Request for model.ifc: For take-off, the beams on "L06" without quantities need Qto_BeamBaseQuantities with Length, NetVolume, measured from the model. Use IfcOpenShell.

First a look at what the model holds.

```python
import ifcopenshell
import ifcopenshell.util.element
import ifcopenshell.util.unit

model = ifcopenshell.open("model.ifc")
print(model.schema)
for unit_type in ("LENGTHUNIT", "AREAUNIT", "VOLUMEUNIT"):
    print(unit_type, ifcopenshell.util.unit.calculate_unit_scale(model, unit_type))
storey = next(s for s in model.by_type("IfcBuildingStorey") if s.Name == "L06")
beams = [e for e in ifcopenshell.util.element.get_decomposition(storey) if e.is_a("IfcBeam")]
for e in sorted(beams, key=lambda e: e.id()):
    print(e.id(), e.is_a(), e.Name, list(ifcopenshell.util.element.get_psets(e, qtos_only=True)), sep=" | ")
```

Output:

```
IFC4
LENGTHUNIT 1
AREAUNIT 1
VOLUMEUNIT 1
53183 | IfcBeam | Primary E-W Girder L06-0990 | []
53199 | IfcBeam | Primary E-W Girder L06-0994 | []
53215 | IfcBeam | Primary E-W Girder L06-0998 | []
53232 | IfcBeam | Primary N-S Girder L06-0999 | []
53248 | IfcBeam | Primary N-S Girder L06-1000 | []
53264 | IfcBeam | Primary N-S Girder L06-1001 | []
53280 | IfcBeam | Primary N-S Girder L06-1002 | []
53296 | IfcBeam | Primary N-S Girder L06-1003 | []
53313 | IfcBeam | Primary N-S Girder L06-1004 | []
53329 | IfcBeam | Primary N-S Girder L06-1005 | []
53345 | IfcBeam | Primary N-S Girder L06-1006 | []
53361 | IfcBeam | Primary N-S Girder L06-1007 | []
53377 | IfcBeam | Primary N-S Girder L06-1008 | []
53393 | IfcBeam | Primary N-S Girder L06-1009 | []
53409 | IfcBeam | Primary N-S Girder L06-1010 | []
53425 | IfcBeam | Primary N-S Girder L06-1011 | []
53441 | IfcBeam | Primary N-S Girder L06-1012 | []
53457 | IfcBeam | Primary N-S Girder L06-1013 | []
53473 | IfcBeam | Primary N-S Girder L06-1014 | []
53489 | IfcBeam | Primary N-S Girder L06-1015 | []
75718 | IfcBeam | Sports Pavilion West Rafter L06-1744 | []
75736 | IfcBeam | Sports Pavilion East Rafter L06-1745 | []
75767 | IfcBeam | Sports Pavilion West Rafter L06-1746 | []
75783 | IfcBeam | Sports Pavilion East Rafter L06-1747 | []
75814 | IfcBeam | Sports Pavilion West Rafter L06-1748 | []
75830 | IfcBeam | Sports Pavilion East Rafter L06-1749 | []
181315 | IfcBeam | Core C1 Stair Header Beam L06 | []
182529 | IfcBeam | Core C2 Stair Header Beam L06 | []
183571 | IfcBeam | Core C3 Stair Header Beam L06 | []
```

```python
import ifcopenshell
import ifcopenshell.api.pset
import ifcopenshell.geom
import ifcopenshell.util.element
import ifcopenshell.util.shape
import ifcopenshell.util.unit

model = ifcopenshell.open("model.ifc")
unit_scale = ifcopenshell.util.unit.calculate_unit_scale(model)
volume_scale = ifcopenshell.util.unit.calculate_unit_scale(model, "VOLUMEUNIT")
settings = ifcopenshell.geom.settings()

storey = next(s for s in model.by_type("IfcBuildingStorey") if s.Name == "L06")
beams = [e for e in ifcopenshell.util.element.get_decomposition(storey) if e.is_a("IfcBeam")]

for e in sorted(beams, key=lambda e: e.id()):
    if ifcopenshell.util.element.get_psets(e, qtos_only=True, should_inherit=False):
        continue
    # Geometry comes back in metres, in the element's own axes.
    shape = ifcopenshell.geom.create_shape(settings, e)
    values = {
        "Length": ifcopenshell.util.shape.get_max_xyz(shape.geometry) / unit_scale,
        "NetVolume": ifcopenshell.util.shape.get_volume(shape.geometry) / volume_scale,
    }
    qto = ifcopenshell.api.pset.add_qto(model, product=e, name="Qto_BeamBaseQuantities")
    ifcopenshell.api.pset.edit_qto(model, qto=qto, properties=values)
    print(e.id(), {k: round(v, 3) for k, v in values.items()})

model.write("model_rev.ifc")
```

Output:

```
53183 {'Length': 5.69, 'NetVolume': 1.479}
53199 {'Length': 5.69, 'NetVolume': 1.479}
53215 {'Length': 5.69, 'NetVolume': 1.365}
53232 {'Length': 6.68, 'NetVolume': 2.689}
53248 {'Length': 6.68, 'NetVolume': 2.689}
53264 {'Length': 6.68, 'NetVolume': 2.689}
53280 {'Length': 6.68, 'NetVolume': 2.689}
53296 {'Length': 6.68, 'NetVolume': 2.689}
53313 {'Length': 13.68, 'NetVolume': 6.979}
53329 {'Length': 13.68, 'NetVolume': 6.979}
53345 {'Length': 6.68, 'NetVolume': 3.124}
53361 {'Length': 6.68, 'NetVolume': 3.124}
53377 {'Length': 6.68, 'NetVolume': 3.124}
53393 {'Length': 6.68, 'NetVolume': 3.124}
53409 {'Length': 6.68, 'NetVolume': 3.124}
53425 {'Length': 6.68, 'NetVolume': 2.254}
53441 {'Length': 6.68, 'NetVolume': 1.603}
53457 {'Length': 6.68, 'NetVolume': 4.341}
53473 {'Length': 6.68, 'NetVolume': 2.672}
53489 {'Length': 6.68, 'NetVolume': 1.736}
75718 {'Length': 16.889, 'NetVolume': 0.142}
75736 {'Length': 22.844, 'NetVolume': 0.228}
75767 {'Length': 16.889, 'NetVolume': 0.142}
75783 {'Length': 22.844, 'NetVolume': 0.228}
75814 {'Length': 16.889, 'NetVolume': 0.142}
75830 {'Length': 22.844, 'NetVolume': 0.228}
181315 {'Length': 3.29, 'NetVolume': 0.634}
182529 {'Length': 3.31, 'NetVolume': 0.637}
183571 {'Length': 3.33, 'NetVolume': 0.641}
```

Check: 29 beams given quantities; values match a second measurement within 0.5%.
